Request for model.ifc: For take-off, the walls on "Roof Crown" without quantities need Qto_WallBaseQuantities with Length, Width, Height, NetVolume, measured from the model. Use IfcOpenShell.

First a look at what the model holds.

```python
import ifcopenshell
import ifcopenshell.util.element
import ifcopenshell.util.unit

model = ifcopenshell.open("model.ifc")
print(model.schema)
for unit_type in ("LENGTHUNIT", "AREAUNIT", "VOLUMEUNIT"):
    print(unit_type, ifcopenshell.util.unit.calculate_unit_scale(model, unit_type))
storey = next(s for s in model.by_type("IfcBuildingStorey") if s.Name == "Roof Crown")
walls = [e for e in ifcopenshell.util.element.get_decomposition(storey) if e.is_a("IfcWall")]
for e in sorted(walls, key=lambda e: e.id()):
    print(e.id(), e.is_a(), e.Name, list(ifcopenshell.util.element.get_psets(e, qtos_only=True)), sep=" | ")
```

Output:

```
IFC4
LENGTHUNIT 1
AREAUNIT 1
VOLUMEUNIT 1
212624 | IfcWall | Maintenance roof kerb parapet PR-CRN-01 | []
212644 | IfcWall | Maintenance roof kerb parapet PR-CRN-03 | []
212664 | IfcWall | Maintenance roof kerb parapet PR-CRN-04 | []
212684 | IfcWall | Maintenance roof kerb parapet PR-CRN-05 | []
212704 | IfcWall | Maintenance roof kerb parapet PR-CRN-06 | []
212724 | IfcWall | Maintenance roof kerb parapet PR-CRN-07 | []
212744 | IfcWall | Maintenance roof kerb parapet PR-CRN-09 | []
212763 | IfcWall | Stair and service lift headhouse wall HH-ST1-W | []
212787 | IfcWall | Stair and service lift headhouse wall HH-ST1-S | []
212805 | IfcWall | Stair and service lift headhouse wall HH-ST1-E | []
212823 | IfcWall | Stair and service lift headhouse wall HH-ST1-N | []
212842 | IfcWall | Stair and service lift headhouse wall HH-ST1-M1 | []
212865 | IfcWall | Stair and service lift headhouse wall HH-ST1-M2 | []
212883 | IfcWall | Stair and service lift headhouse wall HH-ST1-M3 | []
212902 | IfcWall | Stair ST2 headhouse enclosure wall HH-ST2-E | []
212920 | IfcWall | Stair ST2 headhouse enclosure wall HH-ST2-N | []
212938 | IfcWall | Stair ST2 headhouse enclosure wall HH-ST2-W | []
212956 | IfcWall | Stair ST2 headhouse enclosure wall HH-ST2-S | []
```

```python
import ifcopenshell
import ifcopenshell.api.pset
import ifcopenshell.geom
import ifcopenshell.util.element
import ifcopenshell.util.shape
import ifcopenshell.util.unit

model = ifcopenshell.open("model.ifc")
unit_scale = ifcopenshell.util.unit.calculate_unit_scale(model)
volume_scale = ifcopenshell.util.unit.calculate_unit_scale(model, "VOLUMEUNIT")
settings = ifcopenshell.geom.settings()

storey = next(s for s in model.by_type("IfcBuildingStorey") if s.Name == "Roof Crown")
walls = [e for e in ifcopenshell.util.element.get_decomposition(storey) if e.is_a("IfcWall")]

for e in sorted(walls, key=lambda e: e.id()):
    if ifcopenshell.util.element.get_psets(e, qtos_only=True, should_inherit=False):
        continue
    # Geometry comes back in metres, in the element's own axes.
    shape = ifcopenshell.geom.create_shape(settings, e)
    values = {
        "Length": ifcopenshell.util.shape.get_x(shape.geometry) / unit_scale,
        "Width": ifcopenshell.util.shape.get_y(shape.geometry) / unit_scale,
        "Height": ifcopenshell.util.shape.get_z(shape.geometry) / unit_scale,
        "NetVolume": ifcopenshell.util.shape.get_volume(shape.geometry) / volume_scale,
    }
    qto = ifcopenshell.api.pset.add_qto(model, product=e, name="Qto_WallBaseQuantities")
    ifcopenshell.api.pset.edit_qto(model, qto=qto, properties=values)
    print(e.id(), {k: round(v, 3) for k, v in values.items()})

model.write("model_rev.ifc")
```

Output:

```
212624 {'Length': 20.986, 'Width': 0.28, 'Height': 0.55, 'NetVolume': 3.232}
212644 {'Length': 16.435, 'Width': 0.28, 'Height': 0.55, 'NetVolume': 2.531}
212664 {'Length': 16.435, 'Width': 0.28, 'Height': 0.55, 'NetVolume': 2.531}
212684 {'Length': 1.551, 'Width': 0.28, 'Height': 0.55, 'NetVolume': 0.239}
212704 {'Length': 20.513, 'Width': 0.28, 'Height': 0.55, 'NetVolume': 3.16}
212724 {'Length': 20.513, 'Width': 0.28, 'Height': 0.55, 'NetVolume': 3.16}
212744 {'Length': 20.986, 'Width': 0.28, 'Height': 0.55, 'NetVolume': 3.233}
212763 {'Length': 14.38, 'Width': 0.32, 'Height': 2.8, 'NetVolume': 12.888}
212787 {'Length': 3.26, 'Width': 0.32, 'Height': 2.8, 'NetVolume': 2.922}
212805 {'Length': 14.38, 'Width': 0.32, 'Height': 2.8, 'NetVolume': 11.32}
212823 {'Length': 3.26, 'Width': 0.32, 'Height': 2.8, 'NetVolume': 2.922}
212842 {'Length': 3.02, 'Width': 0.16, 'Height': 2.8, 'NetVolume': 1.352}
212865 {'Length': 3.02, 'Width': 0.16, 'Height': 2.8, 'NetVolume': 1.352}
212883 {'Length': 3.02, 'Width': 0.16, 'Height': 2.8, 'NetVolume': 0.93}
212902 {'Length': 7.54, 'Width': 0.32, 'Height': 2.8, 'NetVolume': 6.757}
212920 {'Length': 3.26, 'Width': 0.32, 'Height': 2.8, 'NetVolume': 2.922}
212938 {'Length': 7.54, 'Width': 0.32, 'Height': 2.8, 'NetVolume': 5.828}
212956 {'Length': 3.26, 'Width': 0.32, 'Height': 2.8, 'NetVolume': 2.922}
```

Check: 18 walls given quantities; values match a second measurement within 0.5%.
